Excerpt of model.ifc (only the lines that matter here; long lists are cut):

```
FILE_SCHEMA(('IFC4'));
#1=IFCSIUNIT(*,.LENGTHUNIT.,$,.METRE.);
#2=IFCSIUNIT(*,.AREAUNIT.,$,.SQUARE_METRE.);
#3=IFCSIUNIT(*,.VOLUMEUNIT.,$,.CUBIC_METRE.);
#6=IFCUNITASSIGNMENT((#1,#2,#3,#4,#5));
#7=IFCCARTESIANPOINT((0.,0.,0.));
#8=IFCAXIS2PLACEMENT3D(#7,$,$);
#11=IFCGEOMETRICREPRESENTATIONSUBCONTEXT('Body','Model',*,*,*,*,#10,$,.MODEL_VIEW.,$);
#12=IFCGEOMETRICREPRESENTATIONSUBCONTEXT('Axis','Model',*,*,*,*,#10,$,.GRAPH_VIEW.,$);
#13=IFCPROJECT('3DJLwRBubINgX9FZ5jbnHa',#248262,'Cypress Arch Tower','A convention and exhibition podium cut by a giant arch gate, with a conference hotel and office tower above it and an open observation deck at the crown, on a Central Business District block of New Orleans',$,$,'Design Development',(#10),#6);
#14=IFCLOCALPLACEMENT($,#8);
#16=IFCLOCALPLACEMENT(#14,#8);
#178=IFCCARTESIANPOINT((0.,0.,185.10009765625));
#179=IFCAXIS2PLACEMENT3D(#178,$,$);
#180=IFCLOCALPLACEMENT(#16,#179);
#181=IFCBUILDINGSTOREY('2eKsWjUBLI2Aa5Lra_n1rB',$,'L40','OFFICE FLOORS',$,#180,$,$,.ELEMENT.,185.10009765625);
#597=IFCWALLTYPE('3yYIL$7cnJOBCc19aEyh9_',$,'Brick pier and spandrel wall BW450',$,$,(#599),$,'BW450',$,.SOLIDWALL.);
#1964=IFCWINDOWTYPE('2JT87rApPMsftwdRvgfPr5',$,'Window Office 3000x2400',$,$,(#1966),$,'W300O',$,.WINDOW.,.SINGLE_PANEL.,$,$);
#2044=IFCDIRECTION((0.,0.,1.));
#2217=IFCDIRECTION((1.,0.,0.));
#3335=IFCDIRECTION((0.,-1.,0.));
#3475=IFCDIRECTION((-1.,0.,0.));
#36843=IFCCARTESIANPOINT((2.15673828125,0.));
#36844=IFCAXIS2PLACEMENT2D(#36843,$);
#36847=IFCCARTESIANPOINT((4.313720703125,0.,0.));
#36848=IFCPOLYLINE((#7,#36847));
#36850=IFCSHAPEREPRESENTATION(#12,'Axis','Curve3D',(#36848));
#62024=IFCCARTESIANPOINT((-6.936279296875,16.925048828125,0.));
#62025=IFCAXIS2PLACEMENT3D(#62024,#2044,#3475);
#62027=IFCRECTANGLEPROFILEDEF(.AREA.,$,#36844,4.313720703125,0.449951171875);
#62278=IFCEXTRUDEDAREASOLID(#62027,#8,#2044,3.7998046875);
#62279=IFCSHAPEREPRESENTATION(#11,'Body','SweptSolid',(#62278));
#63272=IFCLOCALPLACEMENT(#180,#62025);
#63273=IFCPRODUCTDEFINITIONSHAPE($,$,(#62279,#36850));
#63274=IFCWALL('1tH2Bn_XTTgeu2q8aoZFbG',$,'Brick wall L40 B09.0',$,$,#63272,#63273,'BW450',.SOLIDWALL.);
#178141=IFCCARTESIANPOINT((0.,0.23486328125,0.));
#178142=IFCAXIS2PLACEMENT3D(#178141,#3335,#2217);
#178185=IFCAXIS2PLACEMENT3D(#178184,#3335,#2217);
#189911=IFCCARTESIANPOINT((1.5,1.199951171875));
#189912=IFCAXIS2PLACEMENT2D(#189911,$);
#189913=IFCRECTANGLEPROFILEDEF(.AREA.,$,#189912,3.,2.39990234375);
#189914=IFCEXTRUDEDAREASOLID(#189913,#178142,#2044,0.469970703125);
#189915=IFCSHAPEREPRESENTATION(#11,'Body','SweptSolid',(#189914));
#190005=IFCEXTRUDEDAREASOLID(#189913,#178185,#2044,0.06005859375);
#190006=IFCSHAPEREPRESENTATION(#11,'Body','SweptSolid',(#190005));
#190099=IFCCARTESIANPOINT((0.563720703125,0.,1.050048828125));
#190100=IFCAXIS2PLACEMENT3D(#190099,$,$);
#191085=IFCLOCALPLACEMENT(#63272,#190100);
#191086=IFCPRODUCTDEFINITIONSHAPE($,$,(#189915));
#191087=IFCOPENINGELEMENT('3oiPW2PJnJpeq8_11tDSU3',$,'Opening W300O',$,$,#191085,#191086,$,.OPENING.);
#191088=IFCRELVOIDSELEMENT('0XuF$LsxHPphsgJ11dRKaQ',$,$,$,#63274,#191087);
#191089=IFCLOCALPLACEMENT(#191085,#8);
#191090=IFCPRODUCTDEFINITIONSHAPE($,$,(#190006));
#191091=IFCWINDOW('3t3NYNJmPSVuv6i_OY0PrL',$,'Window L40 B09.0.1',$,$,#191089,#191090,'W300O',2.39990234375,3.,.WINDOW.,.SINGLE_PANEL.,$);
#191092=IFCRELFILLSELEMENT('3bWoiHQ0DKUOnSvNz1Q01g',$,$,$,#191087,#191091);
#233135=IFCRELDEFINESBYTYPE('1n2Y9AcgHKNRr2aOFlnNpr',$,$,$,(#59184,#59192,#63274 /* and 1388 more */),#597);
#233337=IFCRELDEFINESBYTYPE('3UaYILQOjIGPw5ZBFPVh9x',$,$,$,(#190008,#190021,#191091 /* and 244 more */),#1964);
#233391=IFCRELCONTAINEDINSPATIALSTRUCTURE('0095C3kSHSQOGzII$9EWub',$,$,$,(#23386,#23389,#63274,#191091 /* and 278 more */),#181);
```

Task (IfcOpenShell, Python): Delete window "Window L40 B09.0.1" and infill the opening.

```python
import ifcopenshell
import ifcopenshell.api.feature
import ifcopenshell.api.root
import ifcopenshell.geom
import ifcopenshell.util.shape

model = ifcopenshell.open("model.ifc")
settings = ifcopenshell.geom.settings()


def volume(element):
    """Net volume in cubic metres, openings subtracted."""
    shape = ifcopenshell.geom.create_shape(settings, element)
    return ifcopenshell.util.shape.get_volume(shape.geometry)


window = model.by_guid("3t3NYNJmPSVuv6i_OY0PrL")
opening = window.FillsVoids[0].RelatingOpeningElement
wall = opening.VoidsElements[0].RelatingBuildingElement
before = volume(wall)

ifcopenshell.api.root.remove_product(model, product=window)
ifcopenshell.api.feature.remove_feature(model, feature=opening)

after = volume(wall)

print(f"wall volume {before:.3f} -> {after:.3f} m3")

model.write("model-out.ifc")
```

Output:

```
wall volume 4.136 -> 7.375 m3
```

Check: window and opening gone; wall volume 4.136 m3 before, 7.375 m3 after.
